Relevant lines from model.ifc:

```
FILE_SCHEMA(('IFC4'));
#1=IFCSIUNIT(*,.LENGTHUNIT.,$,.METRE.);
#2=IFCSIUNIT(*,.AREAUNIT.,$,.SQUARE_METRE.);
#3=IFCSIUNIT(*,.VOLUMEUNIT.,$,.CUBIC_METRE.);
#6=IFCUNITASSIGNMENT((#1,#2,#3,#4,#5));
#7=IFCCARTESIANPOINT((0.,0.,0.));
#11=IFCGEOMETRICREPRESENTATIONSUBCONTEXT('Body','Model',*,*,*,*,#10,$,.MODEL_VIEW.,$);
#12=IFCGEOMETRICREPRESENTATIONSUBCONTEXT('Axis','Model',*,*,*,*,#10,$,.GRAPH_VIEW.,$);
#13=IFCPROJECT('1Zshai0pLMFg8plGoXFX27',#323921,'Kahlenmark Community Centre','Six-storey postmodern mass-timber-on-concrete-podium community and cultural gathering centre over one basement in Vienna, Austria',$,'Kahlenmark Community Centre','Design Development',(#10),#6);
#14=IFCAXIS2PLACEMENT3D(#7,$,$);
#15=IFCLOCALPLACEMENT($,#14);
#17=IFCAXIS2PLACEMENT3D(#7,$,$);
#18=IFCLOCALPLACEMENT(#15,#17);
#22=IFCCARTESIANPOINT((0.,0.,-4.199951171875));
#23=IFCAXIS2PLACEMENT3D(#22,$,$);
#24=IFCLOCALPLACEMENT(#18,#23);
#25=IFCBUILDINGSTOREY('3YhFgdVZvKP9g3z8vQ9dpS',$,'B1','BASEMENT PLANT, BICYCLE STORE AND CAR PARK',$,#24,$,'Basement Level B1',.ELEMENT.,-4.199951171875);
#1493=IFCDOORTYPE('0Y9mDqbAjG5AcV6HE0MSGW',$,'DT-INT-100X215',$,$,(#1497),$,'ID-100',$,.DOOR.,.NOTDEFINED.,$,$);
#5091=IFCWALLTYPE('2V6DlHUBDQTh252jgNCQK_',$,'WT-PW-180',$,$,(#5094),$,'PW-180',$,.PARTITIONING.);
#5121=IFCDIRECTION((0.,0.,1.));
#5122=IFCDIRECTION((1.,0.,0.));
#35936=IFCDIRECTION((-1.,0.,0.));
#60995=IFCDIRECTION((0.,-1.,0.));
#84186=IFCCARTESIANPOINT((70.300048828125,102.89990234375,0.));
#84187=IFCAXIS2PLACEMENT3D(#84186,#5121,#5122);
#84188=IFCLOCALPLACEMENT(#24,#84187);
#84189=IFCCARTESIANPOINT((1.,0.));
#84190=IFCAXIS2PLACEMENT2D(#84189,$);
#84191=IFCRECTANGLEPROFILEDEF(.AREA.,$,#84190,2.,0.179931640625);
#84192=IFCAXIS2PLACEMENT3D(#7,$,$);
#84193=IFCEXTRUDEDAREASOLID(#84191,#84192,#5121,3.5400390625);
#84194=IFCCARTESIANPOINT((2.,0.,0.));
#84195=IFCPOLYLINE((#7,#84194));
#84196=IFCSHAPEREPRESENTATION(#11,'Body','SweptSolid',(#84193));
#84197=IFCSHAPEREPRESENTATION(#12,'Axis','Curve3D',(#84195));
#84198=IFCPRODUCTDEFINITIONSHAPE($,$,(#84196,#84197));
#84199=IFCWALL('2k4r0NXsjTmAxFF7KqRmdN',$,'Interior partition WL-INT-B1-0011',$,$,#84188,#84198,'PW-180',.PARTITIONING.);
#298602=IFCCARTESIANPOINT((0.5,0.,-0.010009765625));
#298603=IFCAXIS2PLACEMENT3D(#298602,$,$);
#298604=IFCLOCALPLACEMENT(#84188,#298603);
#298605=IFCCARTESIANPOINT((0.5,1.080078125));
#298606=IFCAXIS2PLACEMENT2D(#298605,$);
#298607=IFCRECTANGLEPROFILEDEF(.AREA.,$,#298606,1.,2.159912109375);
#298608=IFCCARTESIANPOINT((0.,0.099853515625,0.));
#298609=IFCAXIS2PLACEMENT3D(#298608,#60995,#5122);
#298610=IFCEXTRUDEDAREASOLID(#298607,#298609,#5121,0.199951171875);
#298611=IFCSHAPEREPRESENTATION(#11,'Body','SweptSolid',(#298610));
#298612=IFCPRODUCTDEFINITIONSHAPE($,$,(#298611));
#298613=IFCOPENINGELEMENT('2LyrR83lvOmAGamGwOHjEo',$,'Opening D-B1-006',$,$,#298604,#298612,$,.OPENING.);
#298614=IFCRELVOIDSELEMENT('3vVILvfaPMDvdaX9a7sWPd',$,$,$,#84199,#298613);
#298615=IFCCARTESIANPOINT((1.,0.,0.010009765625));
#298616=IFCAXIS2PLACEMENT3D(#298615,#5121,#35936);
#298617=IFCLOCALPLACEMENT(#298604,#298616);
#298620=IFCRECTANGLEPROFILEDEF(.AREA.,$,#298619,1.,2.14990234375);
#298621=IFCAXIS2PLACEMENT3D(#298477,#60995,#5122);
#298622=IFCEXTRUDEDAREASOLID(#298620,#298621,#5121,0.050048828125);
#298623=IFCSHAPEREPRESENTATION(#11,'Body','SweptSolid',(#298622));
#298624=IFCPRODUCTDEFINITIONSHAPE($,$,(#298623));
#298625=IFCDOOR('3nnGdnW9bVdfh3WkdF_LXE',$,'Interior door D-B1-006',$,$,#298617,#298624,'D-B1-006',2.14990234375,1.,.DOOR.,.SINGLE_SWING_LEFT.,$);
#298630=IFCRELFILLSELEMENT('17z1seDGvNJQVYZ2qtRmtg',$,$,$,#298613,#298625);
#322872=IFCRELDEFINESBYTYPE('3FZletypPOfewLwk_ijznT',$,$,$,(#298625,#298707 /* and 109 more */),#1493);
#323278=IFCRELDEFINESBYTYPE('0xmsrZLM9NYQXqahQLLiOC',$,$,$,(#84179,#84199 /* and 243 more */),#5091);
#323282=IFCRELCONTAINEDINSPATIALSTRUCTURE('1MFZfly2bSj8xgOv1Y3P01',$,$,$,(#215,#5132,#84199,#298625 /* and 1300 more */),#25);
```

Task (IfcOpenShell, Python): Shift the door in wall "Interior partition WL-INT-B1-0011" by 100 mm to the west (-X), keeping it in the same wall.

```python
import ifcopenshell
import ifcopenshell.api.geometry
import ifcopenshell.util.placement
import ifcopenshell.util.unit

model = ifcopenshell.open("model.ifc")
unit_scale = ifcopenshell.util.unit.calculate_unit_scale(model)

door = model.by_guid("3nnGdnW9bVdfh3WkdF_LXE")
opening = door.FillsVoids[0].RelatingOpeningElement
wall = opening.VoidsElements[0].RelatingBuildingElement

wall_matrix = ifcopenshell.util.placement.get_local_placement(wall.ObjectPlacement)
shift = wall_matrix[:3, 0] * -0.1 / unit_scale
before = ifcopenshell.util.placement.get_local_placement(door.ObjectPlacement)[:3, 3].copy()

# The door is placed relative to its opening, so it follows when the opening moves.
matrix = ifcopenshell.util.placement.get_local_placement(opening.ObjectPlacement)
matrix[:3, 3] += shift
ifcopenshell.api.geometry.edit_object_placement(
    model, product=opening, matrix=matrix, is_si=False, should_transform_children=True
)

after = ifcopenshell.util.placement.get_local_placement(door.ObjectPlacement)[:3, 3]
print("door moved by", (after - before).round(3) + 0.0)

model.write("model-out.ifc")
```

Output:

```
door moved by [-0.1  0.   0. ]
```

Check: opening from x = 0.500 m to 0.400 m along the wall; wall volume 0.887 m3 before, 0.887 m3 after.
